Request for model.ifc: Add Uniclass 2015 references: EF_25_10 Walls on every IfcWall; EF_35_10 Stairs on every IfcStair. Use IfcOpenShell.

First a look at what the model holds.

```python
import ifcopenshell

model = ifcopenshell.open("model.ifc")
print(model.schema)
print("classifications:", [c.Name for c in model.by_type("IfcClassification")])
for ifc_class in ("IfcDoor", "IfcRoof", "IfcStair", "IfcWall", "IfcWindow"):
    print(ifc_class, len(model.by_type(ifc_class)))
```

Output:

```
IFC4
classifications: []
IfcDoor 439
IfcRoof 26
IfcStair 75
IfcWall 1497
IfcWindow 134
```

```python
import ifcopenshell
import ifcopenshell.api.classification

model = ifcopenshell.open("model.ifc")

system = ifcopenshell.api.classification.add_classification(model, classification="Uniclass 2015")

codes = {
    "IfcWall": ("EF_25_10", "Walls"),
    "IfcStair": ("EF_35_10", "Stairs"),
}
for ifc_class, (code, name) in codes.items():
    products = model.by_type(ifc_class)
    ifcopenshell.api.classification.add_reference(
        model, products=products, classification=system, identification=code, name=name
    )
    print(code, len(products))

model.write("model_updated.ifc")
```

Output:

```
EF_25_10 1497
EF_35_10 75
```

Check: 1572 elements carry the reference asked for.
